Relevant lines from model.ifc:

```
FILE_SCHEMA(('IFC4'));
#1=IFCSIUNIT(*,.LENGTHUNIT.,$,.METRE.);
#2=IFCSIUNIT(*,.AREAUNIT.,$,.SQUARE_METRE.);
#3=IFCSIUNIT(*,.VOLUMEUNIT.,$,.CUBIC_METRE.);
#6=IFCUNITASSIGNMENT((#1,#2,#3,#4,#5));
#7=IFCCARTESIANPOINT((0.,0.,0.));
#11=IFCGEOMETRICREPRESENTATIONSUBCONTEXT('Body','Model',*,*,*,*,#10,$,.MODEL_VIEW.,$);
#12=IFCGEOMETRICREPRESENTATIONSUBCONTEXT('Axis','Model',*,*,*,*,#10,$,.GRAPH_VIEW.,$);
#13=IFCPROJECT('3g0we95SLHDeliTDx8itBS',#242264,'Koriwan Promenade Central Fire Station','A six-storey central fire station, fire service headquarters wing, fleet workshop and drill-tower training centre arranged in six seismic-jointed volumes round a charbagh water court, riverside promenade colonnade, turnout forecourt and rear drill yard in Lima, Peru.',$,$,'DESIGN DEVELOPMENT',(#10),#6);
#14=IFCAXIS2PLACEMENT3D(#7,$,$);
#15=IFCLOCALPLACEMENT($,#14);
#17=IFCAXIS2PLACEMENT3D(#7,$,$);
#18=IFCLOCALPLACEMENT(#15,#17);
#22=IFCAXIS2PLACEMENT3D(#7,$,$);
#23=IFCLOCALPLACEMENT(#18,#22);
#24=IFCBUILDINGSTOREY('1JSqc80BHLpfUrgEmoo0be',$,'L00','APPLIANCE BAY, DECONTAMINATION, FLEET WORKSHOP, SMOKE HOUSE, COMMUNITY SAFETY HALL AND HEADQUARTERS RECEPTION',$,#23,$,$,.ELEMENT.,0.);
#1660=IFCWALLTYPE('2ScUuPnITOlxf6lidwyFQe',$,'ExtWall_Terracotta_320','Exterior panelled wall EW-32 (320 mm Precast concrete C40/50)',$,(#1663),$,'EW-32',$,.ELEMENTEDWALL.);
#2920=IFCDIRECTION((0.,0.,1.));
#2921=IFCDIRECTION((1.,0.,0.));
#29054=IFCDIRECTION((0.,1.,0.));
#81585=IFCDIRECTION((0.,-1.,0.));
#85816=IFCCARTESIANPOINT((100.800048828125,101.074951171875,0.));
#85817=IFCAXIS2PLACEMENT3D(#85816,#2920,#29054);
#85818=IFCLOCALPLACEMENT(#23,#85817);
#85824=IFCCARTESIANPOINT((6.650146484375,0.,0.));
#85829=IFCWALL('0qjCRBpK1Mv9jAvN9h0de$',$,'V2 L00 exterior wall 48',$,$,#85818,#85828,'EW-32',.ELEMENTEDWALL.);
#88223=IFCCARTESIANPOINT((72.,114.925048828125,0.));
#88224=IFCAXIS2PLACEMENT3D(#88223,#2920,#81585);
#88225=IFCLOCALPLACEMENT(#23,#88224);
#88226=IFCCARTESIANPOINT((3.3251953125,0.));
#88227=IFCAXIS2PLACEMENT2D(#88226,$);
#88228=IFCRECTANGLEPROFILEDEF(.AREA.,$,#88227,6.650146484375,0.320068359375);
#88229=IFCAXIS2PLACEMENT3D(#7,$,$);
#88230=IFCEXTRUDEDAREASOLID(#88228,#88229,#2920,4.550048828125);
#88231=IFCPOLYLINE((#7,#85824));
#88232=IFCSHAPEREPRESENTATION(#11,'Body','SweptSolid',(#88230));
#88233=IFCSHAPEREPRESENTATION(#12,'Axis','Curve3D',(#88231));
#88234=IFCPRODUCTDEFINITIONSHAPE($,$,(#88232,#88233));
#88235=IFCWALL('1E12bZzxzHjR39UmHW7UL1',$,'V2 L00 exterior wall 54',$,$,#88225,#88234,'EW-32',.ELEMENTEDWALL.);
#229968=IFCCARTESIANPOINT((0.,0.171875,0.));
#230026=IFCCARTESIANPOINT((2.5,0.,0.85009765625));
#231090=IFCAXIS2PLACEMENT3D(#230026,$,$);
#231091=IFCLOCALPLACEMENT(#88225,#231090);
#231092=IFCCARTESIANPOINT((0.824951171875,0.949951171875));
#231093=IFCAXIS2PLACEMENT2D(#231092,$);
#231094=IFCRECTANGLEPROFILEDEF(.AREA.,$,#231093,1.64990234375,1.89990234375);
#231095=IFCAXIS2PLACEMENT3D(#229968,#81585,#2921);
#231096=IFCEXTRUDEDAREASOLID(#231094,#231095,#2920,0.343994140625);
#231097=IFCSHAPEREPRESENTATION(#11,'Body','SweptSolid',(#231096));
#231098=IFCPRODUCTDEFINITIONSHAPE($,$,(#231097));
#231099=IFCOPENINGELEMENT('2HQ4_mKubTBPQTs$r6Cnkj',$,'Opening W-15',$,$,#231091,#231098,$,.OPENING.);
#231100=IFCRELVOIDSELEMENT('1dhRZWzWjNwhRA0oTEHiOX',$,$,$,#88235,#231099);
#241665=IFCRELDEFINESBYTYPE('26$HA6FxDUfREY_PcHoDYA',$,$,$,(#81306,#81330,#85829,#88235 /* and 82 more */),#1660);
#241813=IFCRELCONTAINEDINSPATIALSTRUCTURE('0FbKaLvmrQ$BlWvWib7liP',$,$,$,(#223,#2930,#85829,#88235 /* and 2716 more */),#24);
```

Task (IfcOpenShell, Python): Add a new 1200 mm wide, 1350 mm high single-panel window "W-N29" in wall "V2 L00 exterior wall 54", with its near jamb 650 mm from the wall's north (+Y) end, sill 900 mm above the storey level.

```python
import numpy as np
import ifcopenshell
import ifcopenshell.api.feature
import ifcopenshell.api.geometry
import ifcopenshell.api.root
import ifcopenshell.api.spatial
import ifcopenshell.geom
import ifcopenshell.util.element
import ifcopenshell.util.placement
import ifcopenshell.util.representation
import ifcopenshell.util.shape
import ifcopenshell.util.unit

model = ifcopenshell.open("model.ifc")
unit_scale = ifcopenshell.util.unit.calculate_unit_scale(model)
settings = ifcopenshell.geom.settings()


def volume(element):
    """Net volume in cubic metres, openings subtracted."""
    shape = ifcopenshell.geom.create_shape(settings, element)
    return ifcopenshell.util.shape.get_volume(shape.geometry)


wall = model.by_guid("1E12bZzxzHjR39UmHW7UL1")
storey = ifcopenshell.util.element.get_container(wall, ifc_class="IfcBuildingStorey")
context = ifcopenshell.util.representation.get_context(model, "Model", "Body", "MODEL_VIEW")
before = volume(wall)

width, height, from_end, sill = 1.2, 1.35, 0.65, 0.9  # metres

# The wall runs along its own X axis, and the end named is its -X end.
wall_shape = ifcopenshell.geom.create_shape(settings, wall)
x, y, z = ifcopenshell.util.shape.get_vertices(wall_shape.geometry).T
start = x.min() + from_end
face, thickness = float(y.min()), float(y.max() - y.min())
wall_matrix = ifcopenshell.util.placement.get_local_placement(wall.ObjectPlacement)
level = ifcopenshell.util.placement.get_local_placement(storey.ObjectPlacement)[2, 3]


def in_wall(x, y):
    """Placement at x, y metres in the wall's axes, at sill height."""
    matrix = wall_matrix.copy()
    matrix[:, 3] = wall_matrix @ np.array([x / unit_scale, y / unit_scale, 0.0, 1.0])
    matrix[2, 3] = level + sill / unit_scale
    return matrix


# Opening: a box that overshoots both wall faces by 50 mm.
opening = ifcopenshell.api.root.create_entity(model, ifc_class="IfcOpeningElement", predefined_type="OPENING")
box = ifcopenshell.api.geometry.add_wall_representation(
    model, context=context, length=width, height=height, thickness=thickness + 0.1
)
ifcopenshell.api.geometry.assign_representation(model, product=opening, representation=box)
ifcopenshell.api.geometry.edit_object_placement(model, product=opening, matrix=in_wall(start, face - 0.05), is_si=False)
ifcopenshell.api.feature.add_feature(model, feature=opening, element=wall)

window = ifcopenshell.api.root.create_entity(model, ifc_class="IfcWindow", name="W-N29", predefined_type="WINDOW")
window.OverallWidth, window.OverallHeight = width / unit_scale, height / unit_scale
window.PartitioningType = "SINGLE_PANEL"
body = ifcopenshell.api.geometry.add_window_representation(
    model,
    context=context,
    overall_width=window.OverallWidth,
    overall_height=window.OverallHeight,
    partition_type="SINGLE_PANEL",
)
ifcopenshell.api.geometry.assign_representation(model, product=window, representation=body)
ifcopenshell.api.spatial.assign_container(model, products=[window], relating_structure=storey)
ifcopenshell.api.feature.add_filling(model, opening=opening, element=window)

# Centre the window in the wall's thickness.
ifcopenshell.api.geometry.edit_object_placement(model, product=window, matrix=in_wall(start, face), is_si=False)
window_shape = ifcopenshell.geom.create_shape(settings, window)
depth = ifcopenshell.util.shape.get_vertices(window_shape.geometry)[:, 1]
offset = face + thickness / 2 - (depth.min() + depth.max()) / 2
ifcopenshell.api.geometry.edit_object_placement(model, product=window, matrix=in_wall(start, offset), is_si=False)

after = volume(wall)

print(f"wall volume {before:.3f} -> {after:.3f} m3")

model.write("model_rev.ifc")
```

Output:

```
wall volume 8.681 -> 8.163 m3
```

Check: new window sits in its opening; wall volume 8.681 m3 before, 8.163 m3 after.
